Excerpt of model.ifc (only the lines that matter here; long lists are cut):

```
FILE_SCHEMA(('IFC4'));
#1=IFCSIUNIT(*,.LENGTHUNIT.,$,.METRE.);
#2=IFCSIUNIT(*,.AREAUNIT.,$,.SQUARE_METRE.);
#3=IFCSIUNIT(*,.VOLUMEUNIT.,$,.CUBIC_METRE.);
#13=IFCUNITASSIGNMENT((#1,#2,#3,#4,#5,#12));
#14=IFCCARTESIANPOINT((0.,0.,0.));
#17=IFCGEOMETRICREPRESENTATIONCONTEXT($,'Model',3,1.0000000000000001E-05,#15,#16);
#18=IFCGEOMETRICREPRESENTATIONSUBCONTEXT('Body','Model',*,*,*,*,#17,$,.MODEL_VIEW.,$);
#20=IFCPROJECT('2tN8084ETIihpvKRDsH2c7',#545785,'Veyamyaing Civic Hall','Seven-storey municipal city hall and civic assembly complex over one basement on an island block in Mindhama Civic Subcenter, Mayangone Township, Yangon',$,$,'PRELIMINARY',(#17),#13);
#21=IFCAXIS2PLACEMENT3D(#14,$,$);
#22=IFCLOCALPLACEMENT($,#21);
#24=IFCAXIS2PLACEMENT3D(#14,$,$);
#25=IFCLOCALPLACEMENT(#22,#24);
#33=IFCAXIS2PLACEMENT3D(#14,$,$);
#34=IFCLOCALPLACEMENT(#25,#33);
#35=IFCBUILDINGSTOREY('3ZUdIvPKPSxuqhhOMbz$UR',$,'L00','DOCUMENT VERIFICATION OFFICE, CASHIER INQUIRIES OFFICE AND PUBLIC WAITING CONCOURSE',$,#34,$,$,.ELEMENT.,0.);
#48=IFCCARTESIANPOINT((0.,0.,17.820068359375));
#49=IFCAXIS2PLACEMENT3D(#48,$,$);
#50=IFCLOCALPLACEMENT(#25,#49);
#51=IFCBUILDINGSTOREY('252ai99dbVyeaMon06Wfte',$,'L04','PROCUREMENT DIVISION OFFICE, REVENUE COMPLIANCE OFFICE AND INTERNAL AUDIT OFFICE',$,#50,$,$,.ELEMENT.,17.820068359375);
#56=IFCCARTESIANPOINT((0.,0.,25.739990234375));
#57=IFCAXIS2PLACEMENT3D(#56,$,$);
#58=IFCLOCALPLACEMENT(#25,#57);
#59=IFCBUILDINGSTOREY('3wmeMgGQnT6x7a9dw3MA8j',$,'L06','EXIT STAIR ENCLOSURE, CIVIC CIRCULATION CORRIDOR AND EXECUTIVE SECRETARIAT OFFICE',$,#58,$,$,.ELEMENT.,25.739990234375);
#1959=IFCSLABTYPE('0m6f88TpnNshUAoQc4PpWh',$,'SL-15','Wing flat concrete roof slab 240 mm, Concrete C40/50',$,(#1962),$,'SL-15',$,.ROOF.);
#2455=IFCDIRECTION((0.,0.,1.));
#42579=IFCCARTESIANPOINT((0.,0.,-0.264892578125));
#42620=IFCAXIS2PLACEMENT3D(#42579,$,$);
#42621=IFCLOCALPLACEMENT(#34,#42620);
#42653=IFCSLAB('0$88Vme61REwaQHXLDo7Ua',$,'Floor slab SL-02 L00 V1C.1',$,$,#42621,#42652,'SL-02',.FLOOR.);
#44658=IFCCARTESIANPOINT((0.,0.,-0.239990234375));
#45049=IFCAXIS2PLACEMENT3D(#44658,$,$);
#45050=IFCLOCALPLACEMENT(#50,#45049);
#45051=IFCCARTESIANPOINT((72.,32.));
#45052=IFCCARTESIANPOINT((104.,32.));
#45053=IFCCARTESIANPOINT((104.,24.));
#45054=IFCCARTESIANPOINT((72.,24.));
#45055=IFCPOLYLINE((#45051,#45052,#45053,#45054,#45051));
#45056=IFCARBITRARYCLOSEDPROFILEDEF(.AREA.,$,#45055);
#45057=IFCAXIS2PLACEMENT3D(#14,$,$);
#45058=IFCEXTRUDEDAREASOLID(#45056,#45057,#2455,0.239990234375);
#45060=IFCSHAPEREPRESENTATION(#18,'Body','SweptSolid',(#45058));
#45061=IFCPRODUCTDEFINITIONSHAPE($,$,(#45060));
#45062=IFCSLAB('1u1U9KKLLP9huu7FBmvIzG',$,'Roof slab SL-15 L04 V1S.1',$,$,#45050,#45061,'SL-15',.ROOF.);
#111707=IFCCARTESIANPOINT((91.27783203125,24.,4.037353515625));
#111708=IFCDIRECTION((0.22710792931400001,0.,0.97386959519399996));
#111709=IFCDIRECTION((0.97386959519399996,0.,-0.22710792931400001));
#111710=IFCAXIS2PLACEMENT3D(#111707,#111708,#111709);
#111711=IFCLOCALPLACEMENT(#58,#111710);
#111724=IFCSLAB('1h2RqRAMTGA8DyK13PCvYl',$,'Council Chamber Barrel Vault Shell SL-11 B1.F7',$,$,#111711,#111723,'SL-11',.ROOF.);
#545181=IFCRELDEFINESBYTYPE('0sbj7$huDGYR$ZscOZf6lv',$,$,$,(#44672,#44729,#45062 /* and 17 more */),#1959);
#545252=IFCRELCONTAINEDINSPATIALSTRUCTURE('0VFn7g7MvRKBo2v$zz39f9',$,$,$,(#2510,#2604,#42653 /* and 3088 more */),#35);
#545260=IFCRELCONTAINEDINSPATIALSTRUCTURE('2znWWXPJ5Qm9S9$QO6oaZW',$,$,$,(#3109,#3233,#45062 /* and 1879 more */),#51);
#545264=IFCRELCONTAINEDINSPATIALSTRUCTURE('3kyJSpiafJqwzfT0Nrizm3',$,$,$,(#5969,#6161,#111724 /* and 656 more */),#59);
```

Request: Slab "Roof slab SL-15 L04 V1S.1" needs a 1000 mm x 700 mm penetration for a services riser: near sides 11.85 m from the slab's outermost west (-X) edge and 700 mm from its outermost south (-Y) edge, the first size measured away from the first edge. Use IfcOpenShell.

```python
import numpy as np
import ifcopenshell
import ifcopenshell.api.feature
import ifcopenshell.api.geometry
import ifcopenshell.api.root
import ifcopenshell.geom
import ifcopenshell.util.placement
import ifcopenshell.util.representation
import ifcopenshell.util.shape
import ifcopenshell.util.unit

model = ifcopenshell.open("model.ifc")
unit_scale = ifcopenshell.util.unit.calculate_unit_scale(model)
settings = ifcopenshell.geom.settings()


def volume(element):
    """Net volume in cubic metres, openings subtracted."""
    shape = ifcopenshell.geom.create_shape(settings, element)
    return ifcopenshell.util.shape.get_volume(shape.geometry)


slab = model.by_id(45062)
before = volume(slab)

# Extent in the slab's own axes, in metres. The edges named are its -X and -Y sides.
slab_shape = ifcopenshell.geom.create_shape(settings, slab)
vertices = ifcopenshell.util.shape.get_vertices(slab_shape.geometry)
x_min, y_min, bottom = vertices.min(axis=0)
top = vertices[:, 2].max()

opening = ifcopenshell.api.root.create_entity(model, ifc_class="IfcOpeningElement", name="Services riser opening", predefined_type="OPENING")
context = ifcopenshell.util.representation.get_context(model, "Model", "Body", "MODEL_VIEW")
width, depth = 1, 0.7
outline = [(0.0, 0.0), (width, 0.0), (width, depth), (0.0, depth), (0.0, 0.0)]
# Overshoot both faces by 50 mm so the cut is clean.
shape = ifcopenshell.api.geometry.add_slab_representation(
    model, context=context, depth=top - bottom + 0.1, polyline=outline
)
ifcopenshell.api.geometry.assign_representation(model, product=opening, representation=shape)

matrix = ifcopenshell.util.placement.get_local_placement(slab.ObjectPlacement)
matrix[:, 3] = matrix @ np.append(np.array([x_min + 11.85, y_min + 0.7, bottom - 0.05]) / unit_scale, 1.0)
ifcopenshell.api.geometry.edit_object_placement(model, product=opening, matrix=matrix, is_si=False)
ifcopenshell.api.feature.add_feature(model, feature=opening, element=slab)

after = volume(slab)

print(f"slab volume {before:.3f} -> {after:.3f} m3")

model.write("model_v2.ifc")
```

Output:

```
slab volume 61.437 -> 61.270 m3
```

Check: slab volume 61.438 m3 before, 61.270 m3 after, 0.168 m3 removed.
